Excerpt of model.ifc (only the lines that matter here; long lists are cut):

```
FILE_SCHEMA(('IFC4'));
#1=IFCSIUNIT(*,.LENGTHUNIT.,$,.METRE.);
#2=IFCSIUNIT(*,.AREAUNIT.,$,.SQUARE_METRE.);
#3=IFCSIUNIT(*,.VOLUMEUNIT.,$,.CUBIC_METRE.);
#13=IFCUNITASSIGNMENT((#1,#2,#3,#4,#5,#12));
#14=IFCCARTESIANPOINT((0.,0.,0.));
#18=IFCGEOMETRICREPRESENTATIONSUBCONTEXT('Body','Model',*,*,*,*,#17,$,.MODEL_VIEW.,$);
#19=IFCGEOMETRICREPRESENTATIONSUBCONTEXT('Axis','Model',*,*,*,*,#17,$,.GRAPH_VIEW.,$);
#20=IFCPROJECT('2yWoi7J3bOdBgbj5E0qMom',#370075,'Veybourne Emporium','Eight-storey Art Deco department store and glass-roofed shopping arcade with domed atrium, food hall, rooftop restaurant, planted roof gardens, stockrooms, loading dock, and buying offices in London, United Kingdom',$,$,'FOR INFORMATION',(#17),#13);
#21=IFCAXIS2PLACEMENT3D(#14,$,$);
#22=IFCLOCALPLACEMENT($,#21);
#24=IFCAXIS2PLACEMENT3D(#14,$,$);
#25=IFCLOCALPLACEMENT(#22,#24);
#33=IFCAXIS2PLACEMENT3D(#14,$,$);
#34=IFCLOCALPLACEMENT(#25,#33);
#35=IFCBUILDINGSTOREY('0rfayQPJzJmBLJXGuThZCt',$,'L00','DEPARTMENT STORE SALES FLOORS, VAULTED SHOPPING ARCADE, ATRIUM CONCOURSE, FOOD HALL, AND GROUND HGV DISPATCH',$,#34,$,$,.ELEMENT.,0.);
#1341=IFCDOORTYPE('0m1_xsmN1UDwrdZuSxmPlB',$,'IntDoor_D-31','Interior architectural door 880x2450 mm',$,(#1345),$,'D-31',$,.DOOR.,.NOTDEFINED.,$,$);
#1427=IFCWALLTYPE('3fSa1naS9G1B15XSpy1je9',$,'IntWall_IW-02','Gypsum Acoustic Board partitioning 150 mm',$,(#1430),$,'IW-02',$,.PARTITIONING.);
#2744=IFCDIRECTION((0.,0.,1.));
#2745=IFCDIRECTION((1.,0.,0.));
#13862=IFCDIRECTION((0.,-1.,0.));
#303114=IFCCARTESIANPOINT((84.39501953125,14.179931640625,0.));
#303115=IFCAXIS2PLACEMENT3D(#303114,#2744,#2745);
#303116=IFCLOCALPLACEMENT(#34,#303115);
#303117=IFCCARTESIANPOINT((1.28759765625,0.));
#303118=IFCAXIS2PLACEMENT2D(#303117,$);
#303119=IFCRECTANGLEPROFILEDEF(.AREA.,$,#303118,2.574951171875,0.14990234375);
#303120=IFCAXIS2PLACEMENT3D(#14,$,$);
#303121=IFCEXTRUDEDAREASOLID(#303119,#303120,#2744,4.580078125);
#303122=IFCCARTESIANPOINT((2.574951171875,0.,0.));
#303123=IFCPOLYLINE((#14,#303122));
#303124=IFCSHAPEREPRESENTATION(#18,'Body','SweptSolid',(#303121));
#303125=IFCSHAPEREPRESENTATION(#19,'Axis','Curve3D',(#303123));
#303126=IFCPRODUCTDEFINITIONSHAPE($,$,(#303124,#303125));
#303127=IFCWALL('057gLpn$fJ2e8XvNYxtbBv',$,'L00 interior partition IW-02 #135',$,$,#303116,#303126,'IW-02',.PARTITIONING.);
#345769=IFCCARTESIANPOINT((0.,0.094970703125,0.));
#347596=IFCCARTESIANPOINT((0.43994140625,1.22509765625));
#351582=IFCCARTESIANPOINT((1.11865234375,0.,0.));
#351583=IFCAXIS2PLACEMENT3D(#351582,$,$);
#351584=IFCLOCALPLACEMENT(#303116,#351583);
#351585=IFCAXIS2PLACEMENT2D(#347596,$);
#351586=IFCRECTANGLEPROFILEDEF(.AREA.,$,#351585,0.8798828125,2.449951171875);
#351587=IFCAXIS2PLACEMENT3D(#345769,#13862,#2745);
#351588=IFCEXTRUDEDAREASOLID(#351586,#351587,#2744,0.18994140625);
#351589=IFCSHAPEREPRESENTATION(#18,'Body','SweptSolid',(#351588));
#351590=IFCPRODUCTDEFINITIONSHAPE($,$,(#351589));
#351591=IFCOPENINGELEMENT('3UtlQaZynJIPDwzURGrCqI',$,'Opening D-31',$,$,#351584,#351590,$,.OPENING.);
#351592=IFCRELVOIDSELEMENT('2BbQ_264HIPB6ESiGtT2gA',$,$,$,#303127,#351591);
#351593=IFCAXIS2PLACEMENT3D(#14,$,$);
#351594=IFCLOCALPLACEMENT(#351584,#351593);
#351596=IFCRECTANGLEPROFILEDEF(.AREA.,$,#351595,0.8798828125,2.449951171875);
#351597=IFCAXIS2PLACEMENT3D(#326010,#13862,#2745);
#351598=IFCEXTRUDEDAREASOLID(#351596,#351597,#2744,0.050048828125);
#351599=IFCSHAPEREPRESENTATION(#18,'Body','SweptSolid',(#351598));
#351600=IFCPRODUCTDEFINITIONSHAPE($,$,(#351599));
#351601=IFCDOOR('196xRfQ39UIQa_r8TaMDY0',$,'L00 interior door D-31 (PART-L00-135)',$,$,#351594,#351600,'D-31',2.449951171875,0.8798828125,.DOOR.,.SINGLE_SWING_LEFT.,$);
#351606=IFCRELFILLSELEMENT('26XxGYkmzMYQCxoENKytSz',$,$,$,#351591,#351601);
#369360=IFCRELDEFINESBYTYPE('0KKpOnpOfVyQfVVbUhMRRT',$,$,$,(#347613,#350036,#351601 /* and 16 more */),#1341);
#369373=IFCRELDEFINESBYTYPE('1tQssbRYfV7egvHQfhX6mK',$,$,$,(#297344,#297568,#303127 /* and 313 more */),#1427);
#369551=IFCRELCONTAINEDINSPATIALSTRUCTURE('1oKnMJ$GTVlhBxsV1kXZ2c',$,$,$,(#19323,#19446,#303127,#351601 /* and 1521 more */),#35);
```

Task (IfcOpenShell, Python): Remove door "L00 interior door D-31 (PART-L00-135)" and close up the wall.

```python
import ifcopenshell
import ifcopenshell.api.feature
import ifcopenshell.api.root
import ifcopenshell.geom
import ifcopenshell.util.shape

model = ifcopenshell.open("model.ifc")
settings = ifcopenshell.geom.settings()


def volume(element):
    """Net volume in cubic metres, openings subtracted."""
    shape = ifcopenshell.geom.create_shape(settings, element)
    return ifcopenshell.util.shape.get_volume(shape.geometry)


door = model.by_guid("196xRfQ39UIQa_r8TaMDY0")
opening = door.FillsVoids[0].RelatingOpeningElement
wall = opening.VoidsElements[0].RelatingBuildingElement
before = volume(wall)

ifcopenshell.api.root.remove_product(model, product=door)
ifcopenshell.api.feature.remove_feature(model, feature=opening)

after = volume(wall)

print(f"wall volume {before:.3f} -> {after:.3f} m3")

model.write("model_updated.ifc")
```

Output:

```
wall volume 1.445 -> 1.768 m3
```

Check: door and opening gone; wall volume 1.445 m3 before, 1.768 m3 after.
